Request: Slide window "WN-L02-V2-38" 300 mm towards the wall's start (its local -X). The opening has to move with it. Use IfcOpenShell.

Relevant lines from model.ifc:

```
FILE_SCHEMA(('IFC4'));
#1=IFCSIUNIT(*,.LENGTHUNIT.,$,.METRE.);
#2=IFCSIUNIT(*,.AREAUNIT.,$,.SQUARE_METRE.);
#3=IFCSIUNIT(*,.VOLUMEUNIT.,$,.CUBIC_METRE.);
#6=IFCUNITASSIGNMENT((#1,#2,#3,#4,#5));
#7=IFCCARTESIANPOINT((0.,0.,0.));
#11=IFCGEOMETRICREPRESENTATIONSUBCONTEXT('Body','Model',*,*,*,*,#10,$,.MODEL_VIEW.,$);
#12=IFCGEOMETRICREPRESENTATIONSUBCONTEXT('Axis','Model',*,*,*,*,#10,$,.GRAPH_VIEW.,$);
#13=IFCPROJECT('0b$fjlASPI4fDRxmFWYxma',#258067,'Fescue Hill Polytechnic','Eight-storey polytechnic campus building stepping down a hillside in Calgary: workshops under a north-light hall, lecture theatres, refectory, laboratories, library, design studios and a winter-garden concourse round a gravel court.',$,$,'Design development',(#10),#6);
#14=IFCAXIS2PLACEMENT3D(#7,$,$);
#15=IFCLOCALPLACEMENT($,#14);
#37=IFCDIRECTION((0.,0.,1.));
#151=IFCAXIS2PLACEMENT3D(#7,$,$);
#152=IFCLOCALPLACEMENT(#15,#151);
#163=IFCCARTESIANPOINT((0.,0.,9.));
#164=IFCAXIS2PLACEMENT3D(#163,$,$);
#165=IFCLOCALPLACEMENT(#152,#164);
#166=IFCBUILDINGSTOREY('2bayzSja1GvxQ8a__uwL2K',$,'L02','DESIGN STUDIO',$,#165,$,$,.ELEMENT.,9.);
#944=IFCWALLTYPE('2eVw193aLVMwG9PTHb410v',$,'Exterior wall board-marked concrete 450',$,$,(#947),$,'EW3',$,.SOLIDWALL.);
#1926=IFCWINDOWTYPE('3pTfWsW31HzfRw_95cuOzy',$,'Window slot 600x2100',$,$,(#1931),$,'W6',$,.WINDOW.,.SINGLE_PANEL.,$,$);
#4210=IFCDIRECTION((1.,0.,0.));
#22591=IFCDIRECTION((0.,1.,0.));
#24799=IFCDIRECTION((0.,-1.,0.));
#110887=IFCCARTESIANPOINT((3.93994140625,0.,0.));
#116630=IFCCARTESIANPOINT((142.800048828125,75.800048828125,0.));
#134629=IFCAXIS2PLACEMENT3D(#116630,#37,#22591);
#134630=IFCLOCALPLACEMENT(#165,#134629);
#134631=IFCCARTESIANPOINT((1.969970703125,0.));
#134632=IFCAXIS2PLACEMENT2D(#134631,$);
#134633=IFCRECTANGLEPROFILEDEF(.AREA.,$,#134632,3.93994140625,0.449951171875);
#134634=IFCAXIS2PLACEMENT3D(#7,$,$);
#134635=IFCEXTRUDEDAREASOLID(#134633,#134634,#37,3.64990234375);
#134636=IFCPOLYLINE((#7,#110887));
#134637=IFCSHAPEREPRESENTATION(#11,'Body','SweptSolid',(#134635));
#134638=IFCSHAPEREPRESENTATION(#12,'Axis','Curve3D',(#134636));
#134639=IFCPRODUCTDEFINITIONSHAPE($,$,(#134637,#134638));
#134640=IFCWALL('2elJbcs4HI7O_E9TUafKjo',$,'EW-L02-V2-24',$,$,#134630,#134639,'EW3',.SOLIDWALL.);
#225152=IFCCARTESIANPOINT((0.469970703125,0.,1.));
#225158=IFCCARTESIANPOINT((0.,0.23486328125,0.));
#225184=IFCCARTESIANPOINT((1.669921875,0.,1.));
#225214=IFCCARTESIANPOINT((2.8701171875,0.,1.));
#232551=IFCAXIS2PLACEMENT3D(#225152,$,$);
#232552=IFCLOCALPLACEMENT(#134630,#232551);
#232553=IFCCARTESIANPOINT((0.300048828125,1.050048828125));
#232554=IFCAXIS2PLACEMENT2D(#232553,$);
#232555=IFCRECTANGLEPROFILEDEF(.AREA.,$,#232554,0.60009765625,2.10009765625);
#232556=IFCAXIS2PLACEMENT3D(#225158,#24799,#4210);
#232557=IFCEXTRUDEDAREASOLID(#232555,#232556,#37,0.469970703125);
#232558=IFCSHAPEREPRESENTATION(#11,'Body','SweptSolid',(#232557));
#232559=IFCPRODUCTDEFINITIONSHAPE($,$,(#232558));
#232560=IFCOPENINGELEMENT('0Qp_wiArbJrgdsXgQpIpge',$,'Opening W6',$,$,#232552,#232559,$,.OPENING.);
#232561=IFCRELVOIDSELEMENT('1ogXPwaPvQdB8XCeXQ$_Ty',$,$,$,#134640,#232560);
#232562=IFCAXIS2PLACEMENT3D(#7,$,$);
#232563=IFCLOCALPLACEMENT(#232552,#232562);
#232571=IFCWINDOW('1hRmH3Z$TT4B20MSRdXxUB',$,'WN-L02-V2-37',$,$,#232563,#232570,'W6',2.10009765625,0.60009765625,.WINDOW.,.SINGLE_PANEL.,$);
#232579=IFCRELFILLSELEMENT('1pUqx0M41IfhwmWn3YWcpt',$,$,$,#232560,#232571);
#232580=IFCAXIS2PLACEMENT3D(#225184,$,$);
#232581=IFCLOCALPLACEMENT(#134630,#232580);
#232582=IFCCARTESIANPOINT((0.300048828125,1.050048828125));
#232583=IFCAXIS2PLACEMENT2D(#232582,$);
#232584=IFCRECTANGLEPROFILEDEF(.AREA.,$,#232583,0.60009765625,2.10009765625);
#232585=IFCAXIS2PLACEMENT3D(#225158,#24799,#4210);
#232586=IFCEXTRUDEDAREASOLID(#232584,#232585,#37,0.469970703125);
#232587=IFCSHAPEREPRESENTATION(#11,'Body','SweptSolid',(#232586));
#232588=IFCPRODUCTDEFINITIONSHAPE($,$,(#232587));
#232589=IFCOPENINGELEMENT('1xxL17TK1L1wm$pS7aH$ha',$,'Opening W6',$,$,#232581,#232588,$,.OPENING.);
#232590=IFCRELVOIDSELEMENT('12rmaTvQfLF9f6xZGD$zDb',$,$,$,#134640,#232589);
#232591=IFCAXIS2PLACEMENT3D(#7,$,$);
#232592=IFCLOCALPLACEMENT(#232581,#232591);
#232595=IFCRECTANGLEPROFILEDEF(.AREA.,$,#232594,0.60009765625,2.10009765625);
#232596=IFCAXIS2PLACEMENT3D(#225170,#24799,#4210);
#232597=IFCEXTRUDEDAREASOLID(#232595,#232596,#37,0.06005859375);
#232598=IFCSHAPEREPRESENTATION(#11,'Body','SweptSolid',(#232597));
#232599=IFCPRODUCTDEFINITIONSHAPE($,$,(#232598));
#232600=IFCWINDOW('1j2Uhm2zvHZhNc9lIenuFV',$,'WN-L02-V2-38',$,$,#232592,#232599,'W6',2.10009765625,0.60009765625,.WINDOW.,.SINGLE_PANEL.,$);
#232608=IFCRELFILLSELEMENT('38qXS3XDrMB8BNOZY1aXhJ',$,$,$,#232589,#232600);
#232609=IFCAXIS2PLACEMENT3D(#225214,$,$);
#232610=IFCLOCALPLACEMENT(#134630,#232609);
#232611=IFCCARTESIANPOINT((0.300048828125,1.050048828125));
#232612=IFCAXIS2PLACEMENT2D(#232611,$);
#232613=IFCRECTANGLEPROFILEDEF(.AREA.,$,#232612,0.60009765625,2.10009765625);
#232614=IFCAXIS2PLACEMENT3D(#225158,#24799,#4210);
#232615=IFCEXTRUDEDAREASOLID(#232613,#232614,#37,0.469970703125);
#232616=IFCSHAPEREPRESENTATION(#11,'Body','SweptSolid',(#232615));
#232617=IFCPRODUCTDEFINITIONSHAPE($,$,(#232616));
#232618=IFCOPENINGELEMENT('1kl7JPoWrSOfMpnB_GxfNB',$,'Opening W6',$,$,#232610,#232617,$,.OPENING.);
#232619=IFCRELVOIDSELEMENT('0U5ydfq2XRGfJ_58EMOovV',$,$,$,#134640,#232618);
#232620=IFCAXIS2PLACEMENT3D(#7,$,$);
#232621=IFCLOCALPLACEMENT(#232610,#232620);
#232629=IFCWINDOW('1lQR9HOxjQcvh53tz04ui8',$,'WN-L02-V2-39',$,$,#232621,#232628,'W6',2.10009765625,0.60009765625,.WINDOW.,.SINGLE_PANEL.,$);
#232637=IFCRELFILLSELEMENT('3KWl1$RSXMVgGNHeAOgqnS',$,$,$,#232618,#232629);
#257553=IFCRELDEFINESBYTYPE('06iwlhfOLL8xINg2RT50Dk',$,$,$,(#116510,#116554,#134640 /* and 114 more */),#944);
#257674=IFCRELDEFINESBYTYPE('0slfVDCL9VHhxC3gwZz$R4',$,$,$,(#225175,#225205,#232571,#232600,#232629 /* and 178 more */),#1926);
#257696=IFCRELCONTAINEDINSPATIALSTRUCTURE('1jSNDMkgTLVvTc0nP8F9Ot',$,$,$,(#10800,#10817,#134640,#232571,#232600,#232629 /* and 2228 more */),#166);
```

```python
import ifcopenshell
import ifcopenshell.api.geometry
import ifcopenshell.util.placement

model = ifcopenshell.open("model.ifc")

window = model.by_id(232600)
opening = window.FillsVoids[0].RelatingOpeningElement
wall = opening.VoidsElements[0].RelatingBuildingElement

wall_matrix = ifcopenshell.util.placement.get_local_placement(wall.ObjectPlacement)
shift = wall_matrix[:3, 0] * -0.3
before = ifcopenshell.util.placement.get_local_placement(window.ObjectPlacement)[:3, 3].copy()

# The window is placed relative to its opening, so it follows when the opening moves.
matrix = ifcopenshell.util.placement.get_local_placement(opening.ObjectPlacement)
matrix[:3, 3] += shift
ifcopenshell.api.geometry.edit_object_placement(
    model, product=opening, matrix=matrix, is_si=False, should_transform_children=True
)

after = ifcopenshell.util.placement.get_local_placement(window.ObjectPlacement)[:3, 3]
print("window moved by", (after - before).round(3) + 0.0)

model.write("model_updated.ifc")
```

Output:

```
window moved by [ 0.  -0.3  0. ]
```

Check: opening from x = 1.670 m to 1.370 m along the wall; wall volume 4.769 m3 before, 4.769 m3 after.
